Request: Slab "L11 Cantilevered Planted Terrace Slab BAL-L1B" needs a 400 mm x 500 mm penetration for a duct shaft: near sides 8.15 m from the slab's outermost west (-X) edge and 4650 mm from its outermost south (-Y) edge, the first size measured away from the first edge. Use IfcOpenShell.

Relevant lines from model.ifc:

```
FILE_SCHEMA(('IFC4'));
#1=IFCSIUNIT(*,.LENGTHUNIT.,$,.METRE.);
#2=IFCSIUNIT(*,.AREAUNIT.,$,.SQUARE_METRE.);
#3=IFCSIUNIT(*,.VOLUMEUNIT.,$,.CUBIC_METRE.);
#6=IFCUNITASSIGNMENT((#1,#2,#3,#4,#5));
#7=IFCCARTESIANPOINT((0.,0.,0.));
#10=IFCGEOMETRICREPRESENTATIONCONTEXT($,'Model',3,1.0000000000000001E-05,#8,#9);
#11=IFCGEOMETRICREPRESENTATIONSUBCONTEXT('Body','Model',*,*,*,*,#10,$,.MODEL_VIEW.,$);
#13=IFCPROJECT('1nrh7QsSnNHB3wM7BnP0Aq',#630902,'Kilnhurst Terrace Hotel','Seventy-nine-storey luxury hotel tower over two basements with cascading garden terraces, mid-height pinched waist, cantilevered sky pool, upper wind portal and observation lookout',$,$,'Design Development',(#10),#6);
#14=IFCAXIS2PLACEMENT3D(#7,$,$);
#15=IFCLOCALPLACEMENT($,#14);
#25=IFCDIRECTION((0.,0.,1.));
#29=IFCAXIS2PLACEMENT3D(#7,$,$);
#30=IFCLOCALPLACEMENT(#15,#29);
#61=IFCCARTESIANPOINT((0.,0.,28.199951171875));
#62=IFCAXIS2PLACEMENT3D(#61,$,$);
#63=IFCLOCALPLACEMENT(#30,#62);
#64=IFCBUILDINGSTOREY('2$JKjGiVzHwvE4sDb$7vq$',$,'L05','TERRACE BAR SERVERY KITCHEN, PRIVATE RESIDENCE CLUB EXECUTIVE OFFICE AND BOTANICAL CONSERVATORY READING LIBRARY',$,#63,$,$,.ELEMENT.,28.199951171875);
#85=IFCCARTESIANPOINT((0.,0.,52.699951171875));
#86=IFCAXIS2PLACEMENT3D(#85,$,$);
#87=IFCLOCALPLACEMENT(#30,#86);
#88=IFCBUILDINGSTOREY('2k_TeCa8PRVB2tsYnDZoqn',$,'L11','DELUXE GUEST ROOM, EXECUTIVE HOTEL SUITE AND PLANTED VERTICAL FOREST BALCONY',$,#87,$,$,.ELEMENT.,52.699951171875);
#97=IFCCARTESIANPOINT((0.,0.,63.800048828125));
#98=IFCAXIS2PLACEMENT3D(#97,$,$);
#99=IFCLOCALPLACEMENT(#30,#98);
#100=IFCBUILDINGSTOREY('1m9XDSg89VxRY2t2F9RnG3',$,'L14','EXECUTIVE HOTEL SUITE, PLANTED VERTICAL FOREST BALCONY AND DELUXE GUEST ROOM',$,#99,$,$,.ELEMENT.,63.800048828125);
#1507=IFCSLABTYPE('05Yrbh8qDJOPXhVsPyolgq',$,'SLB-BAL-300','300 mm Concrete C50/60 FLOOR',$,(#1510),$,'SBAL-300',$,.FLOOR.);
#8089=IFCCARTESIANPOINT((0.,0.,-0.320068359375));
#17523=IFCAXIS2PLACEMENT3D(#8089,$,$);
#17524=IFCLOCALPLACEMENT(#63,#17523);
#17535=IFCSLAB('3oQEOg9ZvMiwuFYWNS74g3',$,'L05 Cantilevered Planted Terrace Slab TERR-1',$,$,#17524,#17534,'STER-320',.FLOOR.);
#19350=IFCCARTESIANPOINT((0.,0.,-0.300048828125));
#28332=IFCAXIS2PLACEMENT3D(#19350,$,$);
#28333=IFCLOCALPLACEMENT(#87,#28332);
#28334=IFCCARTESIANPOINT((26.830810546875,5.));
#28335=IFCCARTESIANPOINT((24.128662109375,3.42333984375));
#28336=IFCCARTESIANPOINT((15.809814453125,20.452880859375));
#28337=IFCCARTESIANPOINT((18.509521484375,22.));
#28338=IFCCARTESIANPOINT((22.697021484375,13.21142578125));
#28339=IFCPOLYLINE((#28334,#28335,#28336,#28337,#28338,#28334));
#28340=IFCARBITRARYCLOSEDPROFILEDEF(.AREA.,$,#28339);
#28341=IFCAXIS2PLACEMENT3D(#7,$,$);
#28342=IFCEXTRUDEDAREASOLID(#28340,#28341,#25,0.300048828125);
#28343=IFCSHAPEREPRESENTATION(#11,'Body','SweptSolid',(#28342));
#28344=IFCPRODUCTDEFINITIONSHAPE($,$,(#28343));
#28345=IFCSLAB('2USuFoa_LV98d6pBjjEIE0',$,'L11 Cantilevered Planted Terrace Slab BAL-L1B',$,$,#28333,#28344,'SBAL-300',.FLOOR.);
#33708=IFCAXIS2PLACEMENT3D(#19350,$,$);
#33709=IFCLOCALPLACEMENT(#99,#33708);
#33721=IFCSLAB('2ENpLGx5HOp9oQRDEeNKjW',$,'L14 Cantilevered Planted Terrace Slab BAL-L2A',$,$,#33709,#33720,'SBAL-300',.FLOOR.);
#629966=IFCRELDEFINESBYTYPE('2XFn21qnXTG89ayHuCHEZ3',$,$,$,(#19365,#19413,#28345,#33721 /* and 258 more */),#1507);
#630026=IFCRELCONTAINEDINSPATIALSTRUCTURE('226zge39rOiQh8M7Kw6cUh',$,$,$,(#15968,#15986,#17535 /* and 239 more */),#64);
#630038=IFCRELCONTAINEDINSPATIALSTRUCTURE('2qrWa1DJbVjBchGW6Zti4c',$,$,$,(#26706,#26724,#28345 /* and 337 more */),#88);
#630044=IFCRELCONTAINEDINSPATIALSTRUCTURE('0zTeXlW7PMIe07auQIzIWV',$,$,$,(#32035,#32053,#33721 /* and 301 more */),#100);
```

```python
import numpy as np
import ifcopenshell
import ifcopenshell.api.feature
import ifcopenshell.api.geometry
import ifcopenshell.api.root
import ifcopenshell.geom
import ifcopenshell.util.placement
import ifcopenshell.util.representation
import ifcopenshell.util.shape
import ifcopenshell.util.unit

model = ifcopenshell.open("model.ifc")
unit_scale = ifcopenshell.util.unit.calculate_unit_scale(model)
settings = ifcopenshell.geom.settings()


def volume(element):
    """Net volume in cubic metres, openings subtracted."""
    shape = ifcopenshell.geom.create_shape(settings, element)
    return ifcopenshell.util.shape.get_volume(shape.geometry)


slab = model.by_guid("2USuFoa_LV98d6pBjjEIE0")
before = volume(slab)

# Extent in the slab's own axes, in metres. The edges named are its -X and -Y sides.
slab_shape = ifcopenshell.geom.create_shape(settings, slab)
vertices = ifcopenshell.util.shape.get_vertices(slab_shape.geometry)
x_min, y_min, bottom = vertices.min(axis=0)
top = vertices[:, 2].max()

opening = ifcopenshell.api.root.create_entity(model, ifc_class="IfcOpeningElement", name="Duct shaft opening", predefined_type="OPENING")
context = ifcopenshell.util.representation.get_context(model, "Model", "Body", "MODEL_VIEW")
width, depth = 0.4, 0.5
outline = [(0.0, 0.0), (width, 0.0), (width, depth), (0.0, depth), (0.0, 0.0)]
# Overshoot both faces by 50 mm so the cut is clean.
shape = ifcopenshell.api.geometry.add_slab_representation(
    model, context=context, depth=top - bottom + 0.1, polyline=outline
)
ifcopenshell.api.geometry.assign_representation(model, product=opening, representation=shape)

matrix = ifcopenshell.util.placement.get_local_placement(slab.ObjectPlacement)
matrix[:, 3] = matrix @ np.append(np.array([x_min + 8.15, y_min + 4.65, bottom - 0.05]) / unit_scale, 1.0)
ifcopenshell.api.geometry.edit_object_placement(model, product=opening, matrix=matrix, is_si=False)
ifcopenshell.api.feature.add_feature(model, feature=opening, element=slab)

after = volume(slab)

print(f"slab volume {before:.3f} -> {after:.3f} m3")

model.write("model_edited.ifc")
```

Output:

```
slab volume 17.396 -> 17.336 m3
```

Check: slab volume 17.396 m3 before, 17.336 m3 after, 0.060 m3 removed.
